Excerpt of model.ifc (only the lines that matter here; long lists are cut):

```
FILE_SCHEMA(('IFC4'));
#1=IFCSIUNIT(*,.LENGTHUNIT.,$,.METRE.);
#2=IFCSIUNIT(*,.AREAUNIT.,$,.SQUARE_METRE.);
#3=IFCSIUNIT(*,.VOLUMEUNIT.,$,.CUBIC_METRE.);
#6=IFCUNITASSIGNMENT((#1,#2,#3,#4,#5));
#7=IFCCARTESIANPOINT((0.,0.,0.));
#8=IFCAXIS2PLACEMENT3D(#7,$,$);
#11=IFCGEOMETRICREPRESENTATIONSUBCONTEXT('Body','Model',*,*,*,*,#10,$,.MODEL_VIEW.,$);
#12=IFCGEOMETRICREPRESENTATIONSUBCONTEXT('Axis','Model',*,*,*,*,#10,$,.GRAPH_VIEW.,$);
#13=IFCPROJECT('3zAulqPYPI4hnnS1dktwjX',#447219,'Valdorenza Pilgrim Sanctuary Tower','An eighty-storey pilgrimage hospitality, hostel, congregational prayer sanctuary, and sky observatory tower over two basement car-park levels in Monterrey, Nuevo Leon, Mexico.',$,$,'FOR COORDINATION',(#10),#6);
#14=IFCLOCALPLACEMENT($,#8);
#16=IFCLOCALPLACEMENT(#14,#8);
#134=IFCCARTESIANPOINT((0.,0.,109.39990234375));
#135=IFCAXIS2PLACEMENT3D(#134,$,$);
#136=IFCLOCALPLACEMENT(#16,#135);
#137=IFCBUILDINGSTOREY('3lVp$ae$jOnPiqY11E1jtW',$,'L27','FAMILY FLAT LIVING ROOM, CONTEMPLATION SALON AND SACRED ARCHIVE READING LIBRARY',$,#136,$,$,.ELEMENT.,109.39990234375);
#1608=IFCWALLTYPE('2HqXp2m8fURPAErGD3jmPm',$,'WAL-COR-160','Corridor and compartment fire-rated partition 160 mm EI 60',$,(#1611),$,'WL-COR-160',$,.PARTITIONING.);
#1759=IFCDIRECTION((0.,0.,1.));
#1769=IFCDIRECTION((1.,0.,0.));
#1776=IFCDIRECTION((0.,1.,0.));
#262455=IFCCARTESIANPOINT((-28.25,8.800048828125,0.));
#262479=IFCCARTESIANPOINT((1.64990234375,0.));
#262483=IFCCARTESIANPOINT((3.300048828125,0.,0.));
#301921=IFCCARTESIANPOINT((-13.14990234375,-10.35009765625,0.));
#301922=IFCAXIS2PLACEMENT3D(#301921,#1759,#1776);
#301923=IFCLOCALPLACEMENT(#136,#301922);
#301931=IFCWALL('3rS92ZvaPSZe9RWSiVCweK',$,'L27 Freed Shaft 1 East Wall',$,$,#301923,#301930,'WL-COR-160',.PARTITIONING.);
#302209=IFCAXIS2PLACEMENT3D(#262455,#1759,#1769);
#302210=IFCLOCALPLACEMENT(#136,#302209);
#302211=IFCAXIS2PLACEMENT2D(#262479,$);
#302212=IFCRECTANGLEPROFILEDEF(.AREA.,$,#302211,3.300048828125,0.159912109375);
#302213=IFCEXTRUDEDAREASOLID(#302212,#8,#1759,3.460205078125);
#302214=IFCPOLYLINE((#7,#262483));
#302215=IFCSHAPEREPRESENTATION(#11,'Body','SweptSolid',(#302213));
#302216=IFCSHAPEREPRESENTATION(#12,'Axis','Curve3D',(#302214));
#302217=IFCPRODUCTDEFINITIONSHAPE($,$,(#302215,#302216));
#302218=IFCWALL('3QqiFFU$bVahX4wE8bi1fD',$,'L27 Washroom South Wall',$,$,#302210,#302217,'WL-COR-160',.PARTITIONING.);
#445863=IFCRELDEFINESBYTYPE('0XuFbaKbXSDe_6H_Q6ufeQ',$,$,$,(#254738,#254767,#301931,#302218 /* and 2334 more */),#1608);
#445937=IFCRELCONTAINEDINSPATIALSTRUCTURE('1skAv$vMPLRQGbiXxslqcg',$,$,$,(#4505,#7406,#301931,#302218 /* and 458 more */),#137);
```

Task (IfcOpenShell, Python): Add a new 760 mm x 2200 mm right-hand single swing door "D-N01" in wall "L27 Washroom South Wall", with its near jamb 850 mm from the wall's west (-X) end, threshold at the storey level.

```python
import numpy as np
import ifcopenshell
import ifcopenshell.api.feature
import ifcopenshell.api.geometry
import ifcopenshell.api.root
import ifcopenshell.api.spatial
import ifcopenshell.geom
import ifcopenshell.util.element
import ifcopenshell.util.placement
import ifcopenshell.util.representation
import ifcopenshell.util.shape
import ifcopenshell.util.unit

model = ifcopenshell.open("model.ifc")
unit_scale = ifcopenshell.util.unit.calculate_unit_scale(model)
settings = ifcopenshell.geom.settings()


def volume(element):
    """Net volume in cubic metres, openings subtracted."""
    shape = ifcopenshell.geom.create_shape(settings, element)
    return ifcopenshell.util.shape.get_volume(shape.geometry)


wall = model.by_id(302218)
storey = ifcopenshell.util.element.get_container(wall, ifc_class="IfcBuildingStorey")
context = ifcopenshell.util.representation.get_context(model, "Model", "Body", "MODEL_VIEW")
before = volume(wall)

width, height, from_end, sill = 0.76, 2.2, 0.85, 0.0  # metres

# The wall runs along its own X axis, and the end named is its -X end.
wall_shape = ifcopenshell.geom.create_shape(settings, wall)
x, y, z = ifcopenshell.util.shape.get_vertices(wall_shape.geometry).T
start = x.min() + from_end
face, thickness = float(y.min()), float(y.max() - y.min())
wall_matrix = ifcopenshell.util.placement.get_local_placement(wall.ObjectPlacement)
level = ifcopenshell.util.placement.get_local_placement(storey.ObjectPlacement)[2, 3]


def in_wall(x, y):
    """Placement at x, y metres in the wall's axes, at sill height."""
    matrix = wall_matrix.copy()
    matrix[:, 3] = wall_matrix @ np.array([x / unit_scale, y / unit_scale, 0.0, 1.0])
    matrix[2, 3] = level + sill / unit_scale
    return matrix


# Opening: a box that overshoots both wall faces by 50 mm.
opening = ifcopenshell.api.root.create_entity(model, ifc_class="IfcOpeningElement", predefined_type="OPENING")
box = ifcopenshell.api.geometry.add_wall_representation(
    model, context=context, length=width, height=height, thickness=thickness + 0.1
)
ifcopenshell.api.geometry.assign_representation(model, product=opening, representation=box)
ifcopenshell.api.geometry.edit_object_placement(model, product=opening, matrix=in_wall(start, face - 0.05), is_si=False)
ifcopenshell.api.feature.add_feature(model, feature=opening, element=wall)

door = ifcopenshell.api.root.create_entity(model, ifc_class="IfcDoor", name="D-N01", predefined_type="DOOR")
door.OverallWidth, door.OverallHeight = width / unit_scale, height / unit_scale
door.OperationType = "SINGLE_SWING_RIGHT"
body = ifcopenshell.api.geometry.add_door_representation(
    model,
    context=context,
    overall_width=door.OverallWidth,
    overall_height=door.OverallHeight,
    operation_type="SINGLE_SWING_RIGHT",
    lining_properties={"LiningDepth": thickness / unit_scale, "ThresholdDepth": thickness / unit_scale},
)
ifcopenshell.api.geometry.assign_representation(model, product=door, representation=body)
ifcopenshell.api.spatial.assign_container(model, products=[door], relating_structure=storey)
ifcopenshell.api.feature.add_filling(model, opening=opening, element=door)

# The lining spans the wall, so the door starts at the wall face.
ifcopenshell.api.geometry.edit_object_placement(model, product=door, matrix=in_wall(start, face), is_si=False)

after = volume(wall)

print(f"wall volume {before:.3f} -> {after:.3f} m3")

model.write("model-out.ifc")
```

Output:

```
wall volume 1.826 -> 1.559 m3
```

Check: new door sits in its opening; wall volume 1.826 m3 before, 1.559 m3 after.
